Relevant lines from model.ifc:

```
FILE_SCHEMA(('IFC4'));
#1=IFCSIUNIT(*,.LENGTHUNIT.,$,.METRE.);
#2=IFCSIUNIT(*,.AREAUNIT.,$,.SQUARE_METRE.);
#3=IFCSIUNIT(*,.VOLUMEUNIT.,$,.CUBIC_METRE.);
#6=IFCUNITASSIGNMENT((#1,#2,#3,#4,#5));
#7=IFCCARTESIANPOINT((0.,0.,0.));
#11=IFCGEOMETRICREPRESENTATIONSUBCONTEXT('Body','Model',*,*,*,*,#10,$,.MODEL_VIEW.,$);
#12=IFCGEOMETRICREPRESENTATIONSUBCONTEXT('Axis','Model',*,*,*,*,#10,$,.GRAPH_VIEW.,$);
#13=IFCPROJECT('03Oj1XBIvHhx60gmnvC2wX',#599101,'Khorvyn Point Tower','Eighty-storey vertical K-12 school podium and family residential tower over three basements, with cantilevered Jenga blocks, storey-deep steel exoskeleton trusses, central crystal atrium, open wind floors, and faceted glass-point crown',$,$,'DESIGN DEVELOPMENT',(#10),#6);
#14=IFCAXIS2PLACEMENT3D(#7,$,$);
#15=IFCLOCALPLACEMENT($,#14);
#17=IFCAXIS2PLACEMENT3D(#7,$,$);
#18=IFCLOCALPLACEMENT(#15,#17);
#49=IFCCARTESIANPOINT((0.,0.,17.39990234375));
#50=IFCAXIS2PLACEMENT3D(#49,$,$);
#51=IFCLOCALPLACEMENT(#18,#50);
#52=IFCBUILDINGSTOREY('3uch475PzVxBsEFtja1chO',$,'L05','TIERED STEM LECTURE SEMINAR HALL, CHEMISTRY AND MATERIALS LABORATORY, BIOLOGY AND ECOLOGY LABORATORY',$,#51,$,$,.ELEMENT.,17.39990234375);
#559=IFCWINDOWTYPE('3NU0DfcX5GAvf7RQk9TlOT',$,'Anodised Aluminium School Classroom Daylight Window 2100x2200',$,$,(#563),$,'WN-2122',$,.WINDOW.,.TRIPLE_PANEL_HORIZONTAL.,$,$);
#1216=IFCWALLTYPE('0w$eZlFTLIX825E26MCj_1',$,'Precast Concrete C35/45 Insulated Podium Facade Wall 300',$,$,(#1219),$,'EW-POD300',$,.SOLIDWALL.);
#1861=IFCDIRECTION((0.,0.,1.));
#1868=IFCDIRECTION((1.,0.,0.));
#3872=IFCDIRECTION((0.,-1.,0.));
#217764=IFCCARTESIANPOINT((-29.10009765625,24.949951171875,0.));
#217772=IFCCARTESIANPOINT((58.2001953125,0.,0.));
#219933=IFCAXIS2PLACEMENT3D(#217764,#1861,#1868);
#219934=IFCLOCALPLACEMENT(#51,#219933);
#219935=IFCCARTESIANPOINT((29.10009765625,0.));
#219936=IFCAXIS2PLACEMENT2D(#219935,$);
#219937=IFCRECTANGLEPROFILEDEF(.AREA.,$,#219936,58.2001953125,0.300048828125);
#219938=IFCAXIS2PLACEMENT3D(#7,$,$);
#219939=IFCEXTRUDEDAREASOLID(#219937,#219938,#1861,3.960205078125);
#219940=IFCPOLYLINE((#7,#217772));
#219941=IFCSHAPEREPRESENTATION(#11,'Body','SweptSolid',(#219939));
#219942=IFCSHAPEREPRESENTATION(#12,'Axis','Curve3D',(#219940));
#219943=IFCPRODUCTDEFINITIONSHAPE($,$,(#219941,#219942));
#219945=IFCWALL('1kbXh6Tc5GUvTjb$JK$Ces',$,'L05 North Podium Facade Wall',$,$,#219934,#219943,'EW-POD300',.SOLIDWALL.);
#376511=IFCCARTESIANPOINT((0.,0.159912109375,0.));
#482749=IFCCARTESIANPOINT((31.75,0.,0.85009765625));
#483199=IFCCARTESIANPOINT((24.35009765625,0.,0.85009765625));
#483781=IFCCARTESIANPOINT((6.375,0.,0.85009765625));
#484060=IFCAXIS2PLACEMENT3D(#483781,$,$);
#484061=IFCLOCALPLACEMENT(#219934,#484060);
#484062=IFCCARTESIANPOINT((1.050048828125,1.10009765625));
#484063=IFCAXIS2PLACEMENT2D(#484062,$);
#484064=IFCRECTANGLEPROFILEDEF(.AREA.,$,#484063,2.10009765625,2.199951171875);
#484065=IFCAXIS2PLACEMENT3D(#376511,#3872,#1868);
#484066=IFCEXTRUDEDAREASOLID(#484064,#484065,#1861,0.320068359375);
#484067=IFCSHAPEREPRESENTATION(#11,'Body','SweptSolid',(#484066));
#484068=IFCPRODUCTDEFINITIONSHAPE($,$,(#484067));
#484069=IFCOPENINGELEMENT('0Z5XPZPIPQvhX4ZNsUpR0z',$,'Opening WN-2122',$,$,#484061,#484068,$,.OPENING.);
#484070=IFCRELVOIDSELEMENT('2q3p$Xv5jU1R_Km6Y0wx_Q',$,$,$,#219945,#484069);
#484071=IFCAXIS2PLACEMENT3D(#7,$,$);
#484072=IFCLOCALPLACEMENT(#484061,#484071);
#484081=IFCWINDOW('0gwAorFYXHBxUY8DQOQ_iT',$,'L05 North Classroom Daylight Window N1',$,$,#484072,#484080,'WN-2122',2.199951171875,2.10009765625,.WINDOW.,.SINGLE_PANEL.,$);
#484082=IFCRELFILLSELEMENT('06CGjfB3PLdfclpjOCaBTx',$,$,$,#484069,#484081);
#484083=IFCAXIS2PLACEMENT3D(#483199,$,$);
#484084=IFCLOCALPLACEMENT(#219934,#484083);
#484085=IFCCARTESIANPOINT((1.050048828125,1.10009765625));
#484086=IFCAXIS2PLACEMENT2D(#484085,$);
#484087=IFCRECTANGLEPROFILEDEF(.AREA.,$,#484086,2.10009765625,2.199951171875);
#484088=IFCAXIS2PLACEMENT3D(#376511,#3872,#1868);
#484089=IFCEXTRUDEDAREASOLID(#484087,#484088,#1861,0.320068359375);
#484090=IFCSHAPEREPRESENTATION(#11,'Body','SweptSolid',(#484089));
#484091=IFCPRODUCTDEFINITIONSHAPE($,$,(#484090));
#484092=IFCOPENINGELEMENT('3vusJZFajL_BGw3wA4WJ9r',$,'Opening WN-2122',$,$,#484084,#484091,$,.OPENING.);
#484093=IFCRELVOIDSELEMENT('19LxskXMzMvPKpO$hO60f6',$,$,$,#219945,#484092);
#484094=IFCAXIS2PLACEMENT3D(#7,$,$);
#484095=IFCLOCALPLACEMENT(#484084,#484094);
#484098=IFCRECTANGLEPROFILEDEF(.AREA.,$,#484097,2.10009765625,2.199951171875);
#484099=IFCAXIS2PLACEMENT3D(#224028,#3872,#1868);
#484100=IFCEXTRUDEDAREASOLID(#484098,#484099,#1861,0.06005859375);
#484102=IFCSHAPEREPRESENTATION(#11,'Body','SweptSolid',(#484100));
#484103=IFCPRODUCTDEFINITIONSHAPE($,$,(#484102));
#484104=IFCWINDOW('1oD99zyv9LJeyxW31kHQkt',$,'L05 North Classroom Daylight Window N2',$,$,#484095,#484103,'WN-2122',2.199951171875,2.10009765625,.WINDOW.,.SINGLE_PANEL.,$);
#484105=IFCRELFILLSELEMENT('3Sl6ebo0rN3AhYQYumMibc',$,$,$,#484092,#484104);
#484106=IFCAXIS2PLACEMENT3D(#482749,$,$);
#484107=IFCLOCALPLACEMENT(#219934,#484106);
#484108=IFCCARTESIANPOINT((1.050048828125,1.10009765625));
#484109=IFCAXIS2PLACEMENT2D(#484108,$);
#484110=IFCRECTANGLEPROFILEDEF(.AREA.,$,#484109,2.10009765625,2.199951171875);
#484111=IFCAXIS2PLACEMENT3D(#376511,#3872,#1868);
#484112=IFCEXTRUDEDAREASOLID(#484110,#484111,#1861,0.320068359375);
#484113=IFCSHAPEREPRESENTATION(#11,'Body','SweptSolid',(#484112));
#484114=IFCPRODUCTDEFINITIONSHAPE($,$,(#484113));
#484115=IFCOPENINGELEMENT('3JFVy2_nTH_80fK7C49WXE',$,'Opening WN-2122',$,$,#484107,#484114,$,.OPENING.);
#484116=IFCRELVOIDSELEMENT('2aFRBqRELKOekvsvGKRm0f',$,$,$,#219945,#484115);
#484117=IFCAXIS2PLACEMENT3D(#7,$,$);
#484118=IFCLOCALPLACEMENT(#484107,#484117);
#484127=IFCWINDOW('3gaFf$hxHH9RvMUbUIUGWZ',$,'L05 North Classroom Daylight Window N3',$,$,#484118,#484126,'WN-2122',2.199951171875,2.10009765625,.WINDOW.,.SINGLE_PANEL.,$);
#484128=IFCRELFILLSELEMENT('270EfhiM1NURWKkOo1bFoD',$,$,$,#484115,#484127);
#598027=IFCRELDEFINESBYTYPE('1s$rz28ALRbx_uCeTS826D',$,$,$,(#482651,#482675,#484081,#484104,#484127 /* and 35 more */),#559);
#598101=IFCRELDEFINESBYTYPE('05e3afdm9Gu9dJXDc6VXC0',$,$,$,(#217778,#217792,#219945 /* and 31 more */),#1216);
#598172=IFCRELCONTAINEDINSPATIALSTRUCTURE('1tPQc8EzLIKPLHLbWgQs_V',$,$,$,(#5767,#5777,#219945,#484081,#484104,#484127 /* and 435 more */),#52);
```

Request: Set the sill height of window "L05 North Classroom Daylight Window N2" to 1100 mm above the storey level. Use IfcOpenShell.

```python
import numpy as np
import ifcopenshell
import ifcopenshell.api.geometry
import ifcopenshell.geom
import ifcopenshell.util.element
import ifcopenshell.util.placement
import ifcopenshell.util.shape
import ifcopenshell.util.unit

model = ifcopenshell.open("model.ifc")
unit_scale = ifcopenshell.util.unit.calculate_unit_scale(model)

window = model.by_id(484104)
opening = window.FillsVoids[0].RelatingOpeningElement
storey = ifcopenshell.util.element.get_container(window, ifc_class="IfcBuildingStorey")
level = ifcopenshell.util.placement.get_local_placement(storey.ObjectPlacement)[2, 3]

# The opening's origin need not be at the sill, so measure its lowest point.
shape = ifcopenshell.geom.create_shape(ifcopenshell.geom.settings(), opening)
bottom = ifcopenshell.util.shape.get_shape_bottom_elevation(shape, shape.geometry) / unit_scale
dz = level + 1.1 / unit_scale - bottom

shift = np.array([0.0, 0.0, dz])
# The window is placed relative to its opening, so it follows when the opening moves.
matrix = ifcopenshell.util.placement.get_local_placement(opening.ObjectPlacement)
matrix[:3, 3] += shift
ifcopenshell.api.geometry.edit_object_placement(
    model, product=opening, matrix=matrix, is_si=False, should_transform_children=True
)

print(f"moved by {dz * unit_scale:+.3f} m")

model.write("model-out.ifc")
```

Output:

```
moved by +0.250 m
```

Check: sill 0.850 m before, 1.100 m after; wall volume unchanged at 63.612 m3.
